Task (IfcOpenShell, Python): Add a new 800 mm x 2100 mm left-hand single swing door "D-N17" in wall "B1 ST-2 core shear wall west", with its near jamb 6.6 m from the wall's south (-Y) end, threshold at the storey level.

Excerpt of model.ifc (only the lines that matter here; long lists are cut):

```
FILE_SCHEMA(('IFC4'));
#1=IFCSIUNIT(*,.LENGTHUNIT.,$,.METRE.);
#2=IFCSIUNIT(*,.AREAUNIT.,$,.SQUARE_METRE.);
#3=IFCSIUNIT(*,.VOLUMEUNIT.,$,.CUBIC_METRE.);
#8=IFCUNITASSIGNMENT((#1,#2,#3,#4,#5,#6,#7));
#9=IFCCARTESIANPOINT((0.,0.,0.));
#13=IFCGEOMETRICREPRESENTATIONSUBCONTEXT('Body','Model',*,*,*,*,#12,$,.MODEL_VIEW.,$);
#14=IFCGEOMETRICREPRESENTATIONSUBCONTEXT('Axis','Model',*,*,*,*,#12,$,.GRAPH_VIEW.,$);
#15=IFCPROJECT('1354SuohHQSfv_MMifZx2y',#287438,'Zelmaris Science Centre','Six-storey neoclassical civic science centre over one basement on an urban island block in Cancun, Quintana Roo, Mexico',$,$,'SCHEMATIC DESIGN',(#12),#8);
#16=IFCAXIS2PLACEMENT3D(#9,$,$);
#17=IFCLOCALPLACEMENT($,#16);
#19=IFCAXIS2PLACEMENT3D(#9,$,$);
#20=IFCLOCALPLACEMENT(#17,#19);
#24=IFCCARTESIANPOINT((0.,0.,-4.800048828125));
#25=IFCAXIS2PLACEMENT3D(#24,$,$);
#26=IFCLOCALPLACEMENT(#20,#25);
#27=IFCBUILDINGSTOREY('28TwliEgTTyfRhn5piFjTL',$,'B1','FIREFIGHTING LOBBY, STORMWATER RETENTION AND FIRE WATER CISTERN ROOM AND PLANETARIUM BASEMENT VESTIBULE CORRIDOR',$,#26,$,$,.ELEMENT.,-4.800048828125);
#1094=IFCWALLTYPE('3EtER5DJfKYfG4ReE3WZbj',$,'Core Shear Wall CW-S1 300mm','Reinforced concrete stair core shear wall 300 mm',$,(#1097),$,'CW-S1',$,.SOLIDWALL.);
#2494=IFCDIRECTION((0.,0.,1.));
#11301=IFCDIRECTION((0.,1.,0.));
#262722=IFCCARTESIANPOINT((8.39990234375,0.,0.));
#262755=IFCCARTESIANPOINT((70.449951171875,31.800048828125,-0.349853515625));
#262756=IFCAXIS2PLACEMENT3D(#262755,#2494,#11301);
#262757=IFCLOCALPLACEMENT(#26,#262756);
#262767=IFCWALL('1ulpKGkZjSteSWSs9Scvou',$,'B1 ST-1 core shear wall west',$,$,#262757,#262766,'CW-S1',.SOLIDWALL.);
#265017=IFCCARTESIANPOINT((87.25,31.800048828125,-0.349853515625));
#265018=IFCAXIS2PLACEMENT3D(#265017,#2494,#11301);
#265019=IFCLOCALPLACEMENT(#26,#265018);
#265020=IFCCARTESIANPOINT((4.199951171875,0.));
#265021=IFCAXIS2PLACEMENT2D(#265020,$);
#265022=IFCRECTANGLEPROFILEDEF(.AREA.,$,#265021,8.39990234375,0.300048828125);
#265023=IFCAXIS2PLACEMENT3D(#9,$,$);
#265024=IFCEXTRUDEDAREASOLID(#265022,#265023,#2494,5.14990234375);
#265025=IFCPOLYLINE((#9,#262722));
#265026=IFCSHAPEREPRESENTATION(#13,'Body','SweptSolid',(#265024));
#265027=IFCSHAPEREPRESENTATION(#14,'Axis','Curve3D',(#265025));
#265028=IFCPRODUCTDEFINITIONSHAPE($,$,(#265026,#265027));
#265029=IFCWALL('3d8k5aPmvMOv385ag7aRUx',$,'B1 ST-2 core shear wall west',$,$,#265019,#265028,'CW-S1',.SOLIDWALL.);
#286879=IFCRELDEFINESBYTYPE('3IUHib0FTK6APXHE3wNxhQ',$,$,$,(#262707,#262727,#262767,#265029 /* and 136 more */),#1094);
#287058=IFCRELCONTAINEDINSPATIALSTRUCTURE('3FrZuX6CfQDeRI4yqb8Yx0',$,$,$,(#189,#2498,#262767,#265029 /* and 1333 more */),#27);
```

```python
import numpy as np
import ifcopenshell
import ifcopenshell.api.feature
import ifcopenshell.api.geometry
import ifcopenshell.api.root
import ifcopenshell.api.spatial
import ifcopenshell.geom
import ifcopenshell.util.element
import ifcopenshell.util.placement
import ifcopenshell.util.representation
import ifcopenshell.util.shape
import ifcopenshell.util.unit

model = ifcopenshell.open("model.ifc")
unit_scale = ifcopenshell.util.unit.calculate_unit_scale(model)
settings = ifcopenshell.geom.settings()


def volume(element):
    """Net volume in cubic metres, openings subtracted."""
    shape = ifcopenshell.geom.create_shape(settings, element)
    return ifcopenshell.util.shape.get_volume(shape.geometry)


wall = model.by_id(265029)
storey = ifcopenshell.util.element.get_container(wall, ifc_class="IfcBuildingStorey")
context = ifcopenshell.util.representation.get_context(model, "Model", "Body", "MODEL_VIEW")
before = volume(wall)

width, height, from_end, sill = 0.8, 2.1, 6.6, 0.0  # metres

# The wall runs along its own X axis, and the end named is its -X end.
wall_shape = ifcopenshell.geom.create_shape(settings, wall)
x, y, z = ifcopenshell.util.shape.get_vertices(wall_shape.geometry).T
start = x.min() + from_end
face, thickness = float(y.min()), float(y.max() - y.min())
wall_matrix = ifcopenshell.util.placement.get_local_placement(wall.ObjectPlacement)
level = ifcopenshell.util.placement.get_local_placement(storey.ObjectPlacement)[2, 3]


def in_wall(x, y):
    """Placement at x, y metres in the wall's axes, at sill height."""
    matrix = wall_matrix.copy()
    matrix[:, 3] = wall_matrix @ np.array([x / unit_scale, y / unit_scale, 0.0, 1.0])
    matrix[2, 3] = level + sill / unit_scale
    return matrix


# Opening: a box that overshoots both wall faces by 50 mm.
opening = ifcopenshell.api.root.create_entity(model, ifc_class="IfcOpeningElement", predefined_type="OPENING")
box = ifcopenshell.api.geometry.add_wall_representation(
    model, context=context, length=width, height=height, thickness=thickness + 0.1
)
ifcopenshell.api.geometry.assign_representation(model, product=opening, representation=box)
ifcopenshell.api.geometry.edit_object_placement(model, product=opening, matrix=in_wall(start, face - 0.05), is_si=False)
ifcopenshell.api.feature.add_feature(model, feature=opening, element=wall)

door = ifcopenshell.api.root.create_entity(model, ifc_class="IfcDoor", name="D-N17", predefined_type="DOOR")
door.OverallWidth, door.OverallHeight = width / unit_scale, height / unit_scale
door.OperationType = "SINGLE_SWING_LEFT"
body = ifcopenshell.api.geometry.add_door_representation(
    model,
    context=context,
    overall_width=door.OverallWidth,
    overall_height=door.OverallHeight,
    operation_type="SINGLE_SWING_LEFT",
    lining_properties={"LiningDepth": thickness / unit_scale, "ThresholdDepth": thickness / unit_scale},
)
ifcopenshell.api.geometry.assign_representation(model, product=door, representation=body)
ifcopenshell.api.spatial.assign_container(model, products=[door], relating_structure=storey)
ifcopenshell.api.feature.add_filling(model, opening=opening, element=door)

# The lining spans the wall, so the door starts at the wall face.
ifcopenshell.api.geometry.edit_object_placement(model, product=door, matrix=in_wall(start, face), is_si=False)

after = volume(wall)

print(f"wall volume {before:.3f} -> {after:.3f} m3")

model.write("model-out.ifc")
```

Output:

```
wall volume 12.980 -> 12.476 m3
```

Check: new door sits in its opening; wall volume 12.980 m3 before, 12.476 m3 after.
